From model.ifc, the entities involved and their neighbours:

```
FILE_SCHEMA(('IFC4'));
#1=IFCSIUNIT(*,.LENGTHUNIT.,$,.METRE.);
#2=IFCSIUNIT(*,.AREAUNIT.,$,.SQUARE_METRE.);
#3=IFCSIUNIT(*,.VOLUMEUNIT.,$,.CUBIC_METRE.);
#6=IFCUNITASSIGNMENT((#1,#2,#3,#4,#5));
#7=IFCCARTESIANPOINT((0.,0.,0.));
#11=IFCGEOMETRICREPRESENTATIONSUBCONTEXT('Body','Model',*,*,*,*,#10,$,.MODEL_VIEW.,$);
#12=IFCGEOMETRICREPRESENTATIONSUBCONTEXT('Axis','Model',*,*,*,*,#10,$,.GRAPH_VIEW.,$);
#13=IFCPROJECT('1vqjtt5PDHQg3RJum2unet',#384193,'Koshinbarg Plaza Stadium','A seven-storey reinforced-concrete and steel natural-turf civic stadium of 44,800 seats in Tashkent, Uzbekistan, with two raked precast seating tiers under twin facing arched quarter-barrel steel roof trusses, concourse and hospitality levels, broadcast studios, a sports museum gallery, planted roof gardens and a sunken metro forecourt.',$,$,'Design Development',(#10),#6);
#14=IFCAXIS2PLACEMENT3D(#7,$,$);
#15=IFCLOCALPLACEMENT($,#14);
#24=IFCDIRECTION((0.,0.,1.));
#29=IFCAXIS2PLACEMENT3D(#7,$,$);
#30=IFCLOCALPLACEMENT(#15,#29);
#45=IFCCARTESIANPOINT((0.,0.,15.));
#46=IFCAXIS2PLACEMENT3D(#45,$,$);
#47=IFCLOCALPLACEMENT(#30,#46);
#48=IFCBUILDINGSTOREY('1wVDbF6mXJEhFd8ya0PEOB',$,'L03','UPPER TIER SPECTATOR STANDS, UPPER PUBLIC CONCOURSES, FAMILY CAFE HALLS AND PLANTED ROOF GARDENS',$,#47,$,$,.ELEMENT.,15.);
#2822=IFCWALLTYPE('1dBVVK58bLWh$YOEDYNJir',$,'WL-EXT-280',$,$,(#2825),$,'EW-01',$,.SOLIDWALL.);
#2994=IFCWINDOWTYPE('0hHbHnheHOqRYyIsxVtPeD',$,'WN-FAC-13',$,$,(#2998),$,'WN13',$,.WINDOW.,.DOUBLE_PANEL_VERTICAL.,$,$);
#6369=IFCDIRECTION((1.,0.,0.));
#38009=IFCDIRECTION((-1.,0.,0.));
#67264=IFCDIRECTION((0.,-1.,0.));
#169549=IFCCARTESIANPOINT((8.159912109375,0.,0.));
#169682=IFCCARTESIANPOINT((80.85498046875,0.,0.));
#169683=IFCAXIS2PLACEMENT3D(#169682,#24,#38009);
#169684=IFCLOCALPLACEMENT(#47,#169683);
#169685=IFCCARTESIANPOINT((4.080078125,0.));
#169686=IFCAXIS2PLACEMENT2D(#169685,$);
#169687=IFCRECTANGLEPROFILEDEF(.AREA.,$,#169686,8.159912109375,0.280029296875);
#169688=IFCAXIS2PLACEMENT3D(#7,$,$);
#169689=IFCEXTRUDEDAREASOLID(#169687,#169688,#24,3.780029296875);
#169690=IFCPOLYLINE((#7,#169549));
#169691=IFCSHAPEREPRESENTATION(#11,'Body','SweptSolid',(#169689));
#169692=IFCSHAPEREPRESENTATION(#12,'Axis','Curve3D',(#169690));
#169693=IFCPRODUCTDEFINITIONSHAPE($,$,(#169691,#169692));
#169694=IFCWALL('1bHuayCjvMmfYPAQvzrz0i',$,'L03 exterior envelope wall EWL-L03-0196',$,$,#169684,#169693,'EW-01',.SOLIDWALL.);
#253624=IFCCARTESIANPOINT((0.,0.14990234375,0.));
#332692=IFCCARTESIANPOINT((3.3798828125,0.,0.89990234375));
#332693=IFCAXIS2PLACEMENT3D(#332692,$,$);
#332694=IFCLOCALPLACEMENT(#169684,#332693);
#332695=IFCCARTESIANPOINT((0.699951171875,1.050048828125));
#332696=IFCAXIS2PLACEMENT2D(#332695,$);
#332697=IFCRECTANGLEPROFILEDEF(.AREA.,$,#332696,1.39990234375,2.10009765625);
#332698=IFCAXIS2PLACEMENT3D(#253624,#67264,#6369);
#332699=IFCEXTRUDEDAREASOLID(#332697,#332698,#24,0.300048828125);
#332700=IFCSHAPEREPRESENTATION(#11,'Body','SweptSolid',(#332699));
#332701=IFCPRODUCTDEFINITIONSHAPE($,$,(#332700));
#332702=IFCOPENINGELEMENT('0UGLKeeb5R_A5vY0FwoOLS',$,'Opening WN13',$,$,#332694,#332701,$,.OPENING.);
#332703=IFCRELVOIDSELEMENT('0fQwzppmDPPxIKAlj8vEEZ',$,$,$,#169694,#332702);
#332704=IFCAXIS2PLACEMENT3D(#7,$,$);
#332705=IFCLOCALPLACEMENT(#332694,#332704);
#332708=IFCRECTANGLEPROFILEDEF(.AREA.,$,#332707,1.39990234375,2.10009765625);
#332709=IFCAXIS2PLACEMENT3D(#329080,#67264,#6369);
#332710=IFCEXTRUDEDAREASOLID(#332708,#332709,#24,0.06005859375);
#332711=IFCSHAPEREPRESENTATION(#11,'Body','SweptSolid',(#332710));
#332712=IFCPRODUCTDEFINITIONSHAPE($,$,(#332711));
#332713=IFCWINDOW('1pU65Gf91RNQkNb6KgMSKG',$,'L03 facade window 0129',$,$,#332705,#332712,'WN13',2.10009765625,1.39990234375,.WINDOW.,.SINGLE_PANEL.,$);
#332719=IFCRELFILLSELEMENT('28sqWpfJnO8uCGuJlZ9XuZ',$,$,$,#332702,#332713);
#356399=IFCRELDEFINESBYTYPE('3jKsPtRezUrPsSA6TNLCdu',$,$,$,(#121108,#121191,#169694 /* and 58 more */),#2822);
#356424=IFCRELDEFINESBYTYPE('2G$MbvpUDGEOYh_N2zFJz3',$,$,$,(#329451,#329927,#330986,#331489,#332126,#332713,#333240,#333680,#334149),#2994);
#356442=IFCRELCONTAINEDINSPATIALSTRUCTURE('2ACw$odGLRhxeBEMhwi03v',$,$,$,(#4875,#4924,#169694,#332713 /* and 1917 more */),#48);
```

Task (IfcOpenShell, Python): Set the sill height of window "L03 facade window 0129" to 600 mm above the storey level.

```python
import numpy as np
import ifcopenshell
import ifcopenshell.api.geometry
import ifcopenshell.geom
import ifcopenshell.util.element
import ifcopenshell.util.placement
import ifcopenshell.util.shape
import ifcopenshell.util.unit

model = ifcopenshell.open("model.ifc")
unit_scale = ifcopenshell.util.unit.calculate_unit_scale(model)

window = model.by_id(332713)
opening = window.FillsVoids[0].RelatingOpeningElement
storey = ifcopenshell.util.element.get_container(window, ifc_class="IfcBuildingStorey")
level = ifcopenshell.util.placement.get_local_placement(storey.ObjectPlacement)[2, 3]

# The opening's origin need not be at the sill, so measure its lowest point.
shape = ifcopenshell.geom.create_shape(ifcopenshell.geom.settings(), opening)
bottom = ifcopenshell.util.shape.get_shape_bottom_elevation(shape, shape.geometry) / unit_scale
dz = level + 0.6 / unit_scale - bottom

shift = np.array([0.0, 0.0, dz])
# The window is placed relative to its opening, so it follows when the opening moves.
matrix = ifcopenshell.util.placement.get_local_placement(opening.ObjectPlacement)
matrix[:3, 3] += shift
ifcopenshell.api.geometry.edit_object_placement(
    model, product=opening, matrix=matrix, is_si=False, should_transform_children=True
)

print(f"moved by {dz * unit_scale:+.3f} m")

model.write("model_v2.ifc")
```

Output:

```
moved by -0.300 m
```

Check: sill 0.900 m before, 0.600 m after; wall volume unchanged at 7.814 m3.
